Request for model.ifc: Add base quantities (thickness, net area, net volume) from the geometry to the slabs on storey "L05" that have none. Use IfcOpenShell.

First a look at what the model holds.

```python
import ifcopenshell
import ifcopenshell.util.element
import ifcopenshell.util.unit

model = ifcopenshell.open("model.ifc")
print(model.schema)
for unit_type in ("LENGTHUNIT", "AREAUNIT", "VOLUMEUNIT"):
    print(unit_type, ifcopenshell.util.unit.calculate_unit_scale(model, unit_type))
storey = next(s for s in model.by_type("IfcBuildingStorey") if s.Name == "L05")
slabs = [e for e in ifcopenshell.util.element.get_decomposition(storey) if e.is_a("IfcSlab")]
for e in sorted(slabs, key=lambda e: e.id()):
    print(e.id(), e.is_a(), e.Name, list(ifcopenshell.util.element.get_psets(e, qtos_only=True)), sep=" | ")
```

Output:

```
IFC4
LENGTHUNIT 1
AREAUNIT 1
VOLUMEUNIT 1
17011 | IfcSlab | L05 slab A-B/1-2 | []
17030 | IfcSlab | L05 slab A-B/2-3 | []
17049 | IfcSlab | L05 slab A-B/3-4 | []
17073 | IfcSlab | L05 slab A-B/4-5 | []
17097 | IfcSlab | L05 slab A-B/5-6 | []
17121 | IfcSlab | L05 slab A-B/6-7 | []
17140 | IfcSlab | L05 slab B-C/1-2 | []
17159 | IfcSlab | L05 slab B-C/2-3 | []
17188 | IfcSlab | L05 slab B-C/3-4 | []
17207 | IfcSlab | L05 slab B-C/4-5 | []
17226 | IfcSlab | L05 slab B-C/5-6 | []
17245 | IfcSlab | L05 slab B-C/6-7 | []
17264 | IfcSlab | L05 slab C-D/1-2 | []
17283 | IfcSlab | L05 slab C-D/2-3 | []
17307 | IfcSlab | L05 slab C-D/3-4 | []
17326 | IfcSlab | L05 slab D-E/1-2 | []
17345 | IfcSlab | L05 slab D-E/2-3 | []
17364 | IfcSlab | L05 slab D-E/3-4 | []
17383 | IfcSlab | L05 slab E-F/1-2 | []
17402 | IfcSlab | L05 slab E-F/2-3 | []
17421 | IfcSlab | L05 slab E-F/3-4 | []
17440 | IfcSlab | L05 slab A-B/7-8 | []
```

```python
import ifcopenshell
import ifcopenshell.api.pset
import ifcopenshell.geom
import ifcopenshell.util.element
import ifcopenshell.util.shape
import ifcopenshell.util.unit

model = ifcopenshell.open("model.ifc")
unit_scale = ifcopenshell.util.unit.calculate_unit_scale(model)
area_scale = ifcopenshell.util.unit.calculate_unit_scale(model, "AREAUNIT")
volume_scale = ifcopenshell.util.unit.calculate_unit_scale(model, "VOLUMEUNIT")
settings = ifcopenshell.geom.settings()

storey = next(s for s in model.by_type("IfcBuildingStorey") if s.Name == "L05")
slabs = [e for e in ifcopenshell.util.element.get_decomposition(storey) if e.is_a("IfcSlab")]

for e in sorted(slabs, key=lambda e: e.id()):
    if ifcopenshell.util.element.get_psets(e, qtos_only=True, should_inherit=False):
        continue
    # Geometry comes back in metres, in the element's own axes.
    shape = ifcopenshell.geom.create_shape(settings, e)
    values = {
        "Width": ifcopenshell.util.shape.get_z(shape.geometry) / unit_scale,
        "NetArea": ifcopenshell.util.shape.get_footprint_area(shape.geometry) / area_scale,
        "NetVolume": ifcopenshell.util.shape.get_volume(shape.geometry) / volume_scale,
    }
    qto = ifcopenshell.api.pset.add_qto(model, product=e, name="Qto_SlabBaseQuantities")
    ifcopenshell.api.pset.edit_qto(model, qto=qto, properties=values)
    print(e.id(), {k: round(v, 3) for k, v in values.items()})

model.write("model_updated.ifc")
```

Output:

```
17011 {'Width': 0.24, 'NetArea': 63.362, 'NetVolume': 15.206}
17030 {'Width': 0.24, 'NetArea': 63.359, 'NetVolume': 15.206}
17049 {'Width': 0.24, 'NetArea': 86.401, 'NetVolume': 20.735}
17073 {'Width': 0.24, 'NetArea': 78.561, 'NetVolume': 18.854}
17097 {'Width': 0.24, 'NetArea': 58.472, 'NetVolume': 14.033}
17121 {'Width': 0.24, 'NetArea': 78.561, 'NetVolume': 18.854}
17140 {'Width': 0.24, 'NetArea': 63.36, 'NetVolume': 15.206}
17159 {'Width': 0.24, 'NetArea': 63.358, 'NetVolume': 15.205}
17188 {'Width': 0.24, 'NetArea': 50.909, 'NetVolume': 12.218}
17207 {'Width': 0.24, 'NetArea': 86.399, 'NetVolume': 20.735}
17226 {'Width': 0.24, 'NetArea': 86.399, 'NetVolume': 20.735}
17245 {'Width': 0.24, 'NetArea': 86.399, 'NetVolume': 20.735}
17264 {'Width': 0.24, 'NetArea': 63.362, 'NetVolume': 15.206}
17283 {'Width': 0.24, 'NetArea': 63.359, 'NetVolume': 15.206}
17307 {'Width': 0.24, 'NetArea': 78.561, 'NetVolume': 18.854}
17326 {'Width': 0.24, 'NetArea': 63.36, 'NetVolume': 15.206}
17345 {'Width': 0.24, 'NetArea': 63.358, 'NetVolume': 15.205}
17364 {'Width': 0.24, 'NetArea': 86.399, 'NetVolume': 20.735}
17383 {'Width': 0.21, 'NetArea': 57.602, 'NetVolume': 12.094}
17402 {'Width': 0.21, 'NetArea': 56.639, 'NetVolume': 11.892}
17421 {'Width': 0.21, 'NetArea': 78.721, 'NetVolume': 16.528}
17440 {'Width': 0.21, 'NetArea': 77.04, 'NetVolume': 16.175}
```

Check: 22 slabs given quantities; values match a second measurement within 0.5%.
